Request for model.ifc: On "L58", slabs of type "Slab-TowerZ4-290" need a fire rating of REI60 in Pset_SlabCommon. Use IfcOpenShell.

First a look at what the model holds.

```python
import ifcopenshell
import ifcopenshell.util.element

model = ifcopenshell.open("model.ifc")
print(model.schema)
storey = next(s for s in model.by_type("IfcBuildingStorey") if s.Name == "L58")
slabs = [e for e in ifcopenshell.util.element.get_decomposition(storey) if e.is_a("IfcSlab")]
seen = {}
for e in slabs:
    element_type = ifcopenshell.util.element.get_type(e)
    key = (element_type.Name if element_type != e and element_type else None, ifcopenshell.util.element.get_pset(e, "Pset_SlabCommon", "FireRating"))
    seen[key] = seen.get(key, 0) + 1
for (name, value), count in sorted(seen.items(), key=str):
    print(count, "x", name, "|", value)
```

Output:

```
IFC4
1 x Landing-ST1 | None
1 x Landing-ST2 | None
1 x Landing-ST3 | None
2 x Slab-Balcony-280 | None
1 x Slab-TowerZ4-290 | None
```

```python
import ifcopenshell
import ifcopenshell.api.pset
import ifcopenshell.util.element

model = ifcopenshell.open("model.ifc")

storey = next(s for s in model.by_type("IfcBuildingStorey") if s.Name == "L58")
slabs = [e for e in ifcopenshell.util.element.get_decomposition(storey) if e.is_a("IfcSlab")]

count = 0
for e in slabs:
    element_type = ifcopenshell.util.element.get_type(e)
    if element_type in (None, e) or element_type.Name != "Slab-TowerZ4-290":
        continue
    found = ifcopenshell.util.element.get_pset(e, "Pset_SlabCommon", should_inherit=False)
    if found:
        pset = model.by_id(found["id"])
        if len(ifcopenshell.util.element.get_elements_by_pset(pset)) > 1:
            pset = ifcopenshell.api.pset.unshare_pset(model, products=[e], pset=pset)[0]
    else:
        pset = ifcopenshell.api.pset.add_pset(model, product=e, name="Pset_SlabCommon")
    ifcopenshell.api.pset.edit_pset(model, pset=pset, properties={"FireRating": "REI60"})
    count += 1

print(count, "slabs updated")

model.write("model-out.ifc")
```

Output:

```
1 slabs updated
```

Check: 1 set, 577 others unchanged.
